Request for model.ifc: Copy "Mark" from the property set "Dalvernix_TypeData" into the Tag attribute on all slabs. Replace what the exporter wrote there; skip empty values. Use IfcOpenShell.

First a look at what the model holds.

```python
import ifcopenshell
import ifcopenshell.util.element

model = ifcopenshell.open("model.ifc")
print(model.schema)
slabs = model.by_type("IfcSlab")
print(len(slabs), "slabs")
for e in slabs[:8]:
    source = ifcopenshell.util.element.get_pset(e, "Dalvernix_TypeData", "Mark")
    target = e.Tag
    print(e.id(), repr(source), repr(target), sep=" | ")
```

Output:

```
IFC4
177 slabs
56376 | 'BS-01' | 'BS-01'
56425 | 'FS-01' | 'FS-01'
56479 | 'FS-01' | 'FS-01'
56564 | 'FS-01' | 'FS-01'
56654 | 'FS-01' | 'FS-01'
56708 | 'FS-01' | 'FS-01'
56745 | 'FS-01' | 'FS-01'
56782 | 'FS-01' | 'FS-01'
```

```python
import ifcopenshell
import ifcopenshell.util.element

model = ifcopenshell.open("model.ifc")

count = 0
for e in model.by_type("IfcSlab"):
    value = ifcopenshell.util.element.get_pset(e, "Dalvernix_TypeData", "Mark")
    current = e.Tag
    if not value or not value.strip() or current == value:
        continue
    e.Tag = value
    count += 1

print(count, "slabs updated")

model.write("model_v2.ifc")
```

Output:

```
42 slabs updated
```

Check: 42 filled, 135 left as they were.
